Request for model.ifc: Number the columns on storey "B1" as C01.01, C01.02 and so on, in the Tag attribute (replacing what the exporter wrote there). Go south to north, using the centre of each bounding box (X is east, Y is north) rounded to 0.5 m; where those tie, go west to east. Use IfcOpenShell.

First a look at what the model holds.

```python
import ifcopenshell
import ifcopenshell.util.element
import ifcopenshell.util.placement

model = ifcopenshell.open("model.ifc")
print(model.schema)
storey = next(s for s in model.by_type("IfcBuildingStorey") if s.Name == "B1")
columns = [e for e in ifcopenshell.util.element.get_decomposition(storey) if e.is_a("IfcColumn")]
for e in sorted(columns, key=lambda e: e.id()):
    origin = ifcopenshell.util.placement.get_local_placement(e.ObjectPlacement)[:3, 3]
    print(e.id(), e.Tag, e.Name, origin.round(2) + 0.0, sep=" | ")
```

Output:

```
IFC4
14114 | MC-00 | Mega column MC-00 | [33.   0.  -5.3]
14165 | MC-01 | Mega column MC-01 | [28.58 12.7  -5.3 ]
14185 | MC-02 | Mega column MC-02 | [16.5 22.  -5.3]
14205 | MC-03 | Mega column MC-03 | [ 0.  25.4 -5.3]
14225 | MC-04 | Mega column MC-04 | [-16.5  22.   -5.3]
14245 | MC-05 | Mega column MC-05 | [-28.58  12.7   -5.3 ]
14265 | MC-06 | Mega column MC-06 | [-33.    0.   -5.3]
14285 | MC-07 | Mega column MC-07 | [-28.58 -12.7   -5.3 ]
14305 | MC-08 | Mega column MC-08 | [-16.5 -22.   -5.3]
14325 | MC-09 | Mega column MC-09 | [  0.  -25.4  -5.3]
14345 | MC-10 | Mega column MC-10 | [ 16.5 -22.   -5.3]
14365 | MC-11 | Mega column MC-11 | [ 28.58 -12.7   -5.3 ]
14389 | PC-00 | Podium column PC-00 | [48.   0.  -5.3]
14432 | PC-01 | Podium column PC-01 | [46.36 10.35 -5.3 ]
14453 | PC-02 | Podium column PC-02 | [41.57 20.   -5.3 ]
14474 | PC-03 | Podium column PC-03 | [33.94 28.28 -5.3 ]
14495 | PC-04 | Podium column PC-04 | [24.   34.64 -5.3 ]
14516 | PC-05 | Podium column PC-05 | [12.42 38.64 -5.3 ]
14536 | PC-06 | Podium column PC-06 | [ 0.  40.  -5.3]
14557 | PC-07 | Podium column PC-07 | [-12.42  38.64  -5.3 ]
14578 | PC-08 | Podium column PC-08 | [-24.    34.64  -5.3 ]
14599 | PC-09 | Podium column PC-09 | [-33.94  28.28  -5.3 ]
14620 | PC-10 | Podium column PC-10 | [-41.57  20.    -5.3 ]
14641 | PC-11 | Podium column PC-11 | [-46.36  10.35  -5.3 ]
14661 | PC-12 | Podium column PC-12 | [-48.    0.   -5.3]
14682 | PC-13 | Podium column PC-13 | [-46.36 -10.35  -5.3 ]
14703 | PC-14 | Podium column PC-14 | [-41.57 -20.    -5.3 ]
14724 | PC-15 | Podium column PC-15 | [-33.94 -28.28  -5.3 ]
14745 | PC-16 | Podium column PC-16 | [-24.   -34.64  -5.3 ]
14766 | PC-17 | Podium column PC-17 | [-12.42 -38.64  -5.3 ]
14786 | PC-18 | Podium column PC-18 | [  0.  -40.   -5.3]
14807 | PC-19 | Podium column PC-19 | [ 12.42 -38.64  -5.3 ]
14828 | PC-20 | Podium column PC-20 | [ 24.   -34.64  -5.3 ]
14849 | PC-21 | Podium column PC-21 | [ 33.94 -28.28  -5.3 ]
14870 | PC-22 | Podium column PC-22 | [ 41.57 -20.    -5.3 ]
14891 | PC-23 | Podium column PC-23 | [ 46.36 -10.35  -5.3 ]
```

```python
import ifcopenshell
import ifcopenshell.geom
import ifcopenshell.util.element
import ifcopenshell.util.shape

model = ifcopenshell.open("model.ifc")
settings = ifcopenshell.geom.settings()
settings.set("use-world-coords", True)


def centre(element):
    shape = ifcopenshell.geom.create_shape(settings, element)
    return ifcopenshell.util.shape.get_bbox_centroid(shape.geometry)


storey = next(s for s in model.by_type("IfcBuildingStorey") if s.Name == "B1")
columns = [e for e in ifcopenshell.util.element.get_decomposition(storey) if e.is_a("IfcColumn")]

# Insertion points can sit at a corner or the storey origin, so sort by the geometry (in metres).
centres = {e: centre(e) for e in columns}
columns.sort(key=lambda e: (round(centres[e][1] / 0.5), centres[e][0]))

for i, e in enumerate(columns, start=1):
    number = f"C01.{i:02d}"
    e.Tag = number
    print(e.id(), number)

model.write("model_updated.ifc")
```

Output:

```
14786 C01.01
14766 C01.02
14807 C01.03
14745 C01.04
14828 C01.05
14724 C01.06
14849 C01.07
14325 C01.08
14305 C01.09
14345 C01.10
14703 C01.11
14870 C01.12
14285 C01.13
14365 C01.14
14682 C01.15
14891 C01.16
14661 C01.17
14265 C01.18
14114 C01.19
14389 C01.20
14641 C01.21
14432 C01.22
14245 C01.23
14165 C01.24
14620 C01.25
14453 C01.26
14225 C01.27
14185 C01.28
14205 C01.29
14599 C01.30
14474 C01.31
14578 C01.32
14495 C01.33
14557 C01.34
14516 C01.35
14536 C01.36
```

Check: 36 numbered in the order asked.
